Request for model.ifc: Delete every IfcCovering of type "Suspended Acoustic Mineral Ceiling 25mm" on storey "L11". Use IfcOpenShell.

First a look at what the model holds.

```python
import ifcopenshell
import ifcopenshell.util.element

model = ifcopenshell.open("model.ifc")
print(model.schema)
storey = next(s for s in model.by_type("IfcBuildingStorey") if s.Name == "L11")
coverings = [e for e in ifcopenshell.util.element.get_decomposition(storey) if e.is_a("IfcCovering")]
seen = {}
for e in coverings:
    element_type = ifcopenshell.util.element.get_type(e)
    name = element_type.Name if element_type not in (None, e) else None
    seen[name] = seen.get(name, 0) + 1
for name, count in sorted(seen.items(), key=str):
    print(count, "x", name)
```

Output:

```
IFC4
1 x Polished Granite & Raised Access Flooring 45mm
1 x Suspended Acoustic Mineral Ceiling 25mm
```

```python
import ifcopenshell
import ifcopenshell.api.root
import ifcopenshell.util.element

model = ifcopenshell.open("model.ifc")

storey = next(s for s in model.by_type("IfcBuildingStorey") if s.Name == "L11")
coverings = [e for e in ifcopenshell.util.element.get_decomposition(storey) if e.is_a("IfcCovering")]
targets = [e for e in coverings if (t := ifcopenshell.util.element.get_type(e)) not in (None, e) and t.Name == "Suspended Acoustic Mineral Ceiling 25mm"]

for e in targets:
    ifcopenshell.api.root.remove_product(model, product=e)
print(len(targets), "removed")

model.write("model_rev.ifc")
```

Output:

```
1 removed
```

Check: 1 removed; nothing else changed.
